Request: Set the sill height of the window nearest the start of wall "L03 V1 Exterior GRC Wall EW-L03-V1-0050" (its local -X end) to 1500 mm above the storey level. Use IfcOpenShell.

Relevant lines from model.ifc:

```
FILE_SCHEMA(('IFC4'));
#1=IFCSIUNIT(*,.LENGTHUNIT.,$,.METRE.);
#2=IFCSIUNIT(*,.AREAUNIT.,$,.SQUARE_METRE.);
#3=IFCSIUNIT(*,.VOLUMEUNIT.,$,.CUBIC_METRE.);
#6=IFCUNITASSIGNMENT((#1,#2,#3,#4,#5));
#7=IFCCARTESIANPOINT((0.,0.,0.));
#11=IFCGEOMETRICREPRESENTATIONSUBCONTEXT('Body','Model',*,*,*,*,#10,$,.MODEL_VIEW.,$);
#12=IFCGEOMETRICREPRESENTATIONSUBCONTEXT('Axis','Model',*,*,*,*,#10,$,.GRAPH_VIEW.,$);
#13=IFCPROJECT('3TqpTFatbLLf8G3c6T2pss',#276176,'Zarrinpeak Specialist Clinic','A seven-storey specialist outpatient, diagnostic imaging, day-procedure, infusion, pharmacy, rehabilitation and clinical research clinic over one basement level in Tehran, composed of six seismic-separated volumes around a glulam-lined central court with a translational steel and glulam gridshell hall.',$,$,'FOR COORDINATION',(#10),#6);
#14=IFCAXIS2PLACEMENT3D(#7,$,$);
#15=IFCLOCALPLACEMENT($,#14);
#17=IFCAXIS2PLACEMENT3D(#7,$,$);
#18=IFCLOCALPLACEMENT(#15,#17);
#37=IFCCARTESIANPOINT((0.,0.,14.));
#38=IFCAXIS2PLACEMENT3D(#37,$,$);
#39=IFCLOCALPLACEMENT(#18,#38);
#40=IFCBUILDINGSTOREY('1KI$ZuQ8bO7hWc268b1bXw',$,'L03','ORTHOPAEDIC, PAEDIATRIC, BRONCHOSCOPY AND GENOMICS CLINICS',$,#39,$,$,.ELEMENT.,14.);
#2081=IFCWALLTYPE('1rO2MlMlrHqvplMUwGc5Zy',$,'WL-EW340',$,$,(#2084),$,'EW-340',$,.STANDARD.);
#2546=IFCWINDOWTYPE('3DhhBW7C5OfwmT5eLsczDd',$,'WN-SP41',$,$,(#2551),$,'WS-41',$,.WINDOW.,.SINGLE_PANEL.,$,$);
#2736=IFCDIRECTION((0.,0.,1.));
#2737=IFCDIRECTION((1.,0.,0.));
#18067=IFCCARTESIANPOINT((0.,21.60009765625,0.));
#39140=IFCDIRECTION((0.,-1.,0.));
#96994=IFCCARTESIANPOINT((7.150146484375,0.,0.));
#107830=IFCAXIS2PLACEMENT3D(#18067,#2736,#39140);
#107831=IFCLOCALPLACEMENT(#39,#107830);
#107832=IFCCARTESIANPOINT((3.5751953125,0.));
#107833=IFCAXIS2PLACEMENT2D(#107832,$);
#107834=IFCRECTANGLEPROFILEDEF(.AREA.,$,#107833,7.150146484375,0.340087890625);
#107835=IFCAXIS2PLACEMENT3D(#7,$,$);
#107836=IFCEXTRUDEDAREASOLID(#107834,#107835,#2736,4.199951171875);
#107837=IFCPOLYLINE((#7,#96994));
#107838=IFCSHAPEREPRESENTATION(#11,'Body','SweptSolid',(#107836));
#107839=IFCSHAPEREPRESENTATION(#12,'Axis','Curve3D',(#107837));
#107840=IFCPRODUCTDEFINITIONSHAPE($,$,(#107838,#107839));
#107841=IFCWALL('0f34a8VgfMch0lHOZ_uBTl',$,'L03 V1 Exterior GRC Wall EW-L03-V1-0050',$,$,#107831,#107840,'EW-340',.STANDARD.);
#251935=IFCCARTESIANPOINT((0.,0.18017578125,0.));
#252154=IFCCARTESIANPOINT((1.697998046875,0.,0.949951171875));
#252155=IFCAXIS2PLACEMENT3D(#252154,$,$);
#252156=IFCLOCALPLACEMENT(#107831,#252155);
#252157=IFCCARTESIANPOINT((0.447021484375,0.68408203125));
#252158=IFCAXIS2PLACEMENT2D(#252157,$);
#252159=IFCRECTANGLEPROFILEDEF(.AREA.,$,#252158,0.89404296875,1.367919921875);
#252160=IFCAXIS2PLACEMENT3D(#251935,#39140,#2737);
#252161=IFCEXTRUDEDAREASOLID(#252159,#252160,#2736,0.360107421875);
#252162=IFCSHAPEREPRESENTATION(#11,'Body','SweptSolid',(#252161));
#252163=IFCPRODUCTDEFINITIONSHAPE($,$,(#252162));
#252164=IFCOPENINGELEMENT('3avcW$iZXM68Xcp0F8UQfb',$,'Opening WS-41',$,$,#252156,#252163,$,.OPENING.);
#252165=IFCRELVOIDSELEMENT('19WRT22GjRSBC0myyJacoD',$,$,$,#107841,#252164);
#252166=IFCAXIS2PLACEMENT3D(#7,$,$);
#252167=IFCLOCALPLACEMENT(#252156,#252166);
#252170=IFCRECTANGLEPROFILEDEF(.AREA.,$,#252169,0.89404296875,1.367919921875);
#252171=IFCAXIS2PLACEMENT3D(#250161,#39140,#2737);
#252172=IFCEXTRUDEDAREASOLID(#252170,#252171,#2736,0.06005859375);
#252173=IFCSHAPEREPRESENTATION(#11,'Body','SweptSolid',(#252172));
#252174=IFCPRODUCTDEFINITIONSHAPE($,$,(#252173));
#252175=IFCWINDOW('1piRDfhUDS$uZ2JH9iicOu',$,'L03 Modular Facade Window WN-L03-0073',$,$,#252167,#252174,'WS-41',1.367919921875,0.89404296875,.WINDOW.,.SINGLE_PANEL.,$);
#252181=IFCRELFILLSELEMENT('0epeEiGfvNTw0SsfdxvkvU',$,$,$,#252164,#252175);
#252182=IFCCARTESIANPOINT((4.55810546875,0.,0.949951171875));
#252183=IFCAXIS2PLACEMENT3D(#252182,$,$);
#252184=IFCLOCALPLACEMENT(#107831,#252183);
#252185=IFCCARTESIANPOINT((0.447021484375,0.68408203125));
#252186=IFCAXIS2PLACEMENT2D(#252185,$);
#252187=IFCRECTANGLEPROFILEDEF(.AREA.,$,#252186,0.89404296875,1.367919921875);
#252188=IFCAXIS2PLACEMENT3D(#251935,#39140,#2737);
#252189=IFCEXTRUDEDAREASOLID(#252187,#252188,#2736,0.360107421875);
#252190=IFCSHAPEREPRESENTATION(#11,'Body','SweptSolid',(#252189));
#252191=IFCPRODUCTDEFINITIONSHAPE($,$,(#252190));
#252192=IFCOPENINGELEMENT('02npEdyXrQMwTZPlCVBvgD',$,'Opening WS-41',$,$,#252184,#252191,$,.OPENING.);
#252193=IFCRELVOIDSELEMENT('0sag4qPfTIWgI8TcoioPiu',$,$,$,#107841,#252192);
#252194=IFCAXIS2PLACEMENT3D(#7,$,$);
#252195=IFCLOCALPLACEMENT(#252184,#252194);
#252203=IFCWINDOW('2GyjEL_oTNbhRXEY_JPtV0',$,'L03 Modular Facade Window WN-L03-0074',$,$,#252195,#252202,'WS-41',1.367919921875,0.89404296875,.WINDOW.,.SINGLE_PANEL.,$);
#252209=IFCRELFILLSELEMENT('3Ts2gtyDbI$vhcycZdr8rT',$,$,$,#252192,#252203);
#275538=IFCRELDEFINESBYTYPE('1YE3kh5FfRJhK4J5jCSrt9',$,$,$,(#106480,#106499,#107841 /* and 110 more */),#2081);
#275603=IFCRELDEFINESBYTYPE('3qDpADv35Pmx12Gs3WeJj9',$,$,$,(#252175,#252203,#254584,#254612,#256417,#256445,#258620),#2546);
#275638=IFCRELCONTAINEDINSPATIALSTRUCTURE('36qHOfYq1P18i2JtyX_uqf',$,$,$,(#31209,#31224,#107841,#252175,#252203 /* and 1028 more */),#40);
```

```python
import numpy as np
import ifcopenshell
import ifcopenshell.api.geometry
import ifcopenshell.geom
import ifcopenshell.util.element
import ifcopenshell.util.placement
import ifcopenshell.util.shape
import ifcopenshell.util.unit

model = ifcopenshell.open("model.ifc")
unit_scale = ifcopenshell.util.unit.calculate_unit_scale(model)

window = model.by_guid("1piRDfhUDS$uZ2JH9iicOu")
opening = window.FillsVoids[0].RelatingOpeningElement
storey = ifcopenshell.util.element.get_container(window, ifc_class="IfcBuildingStorey")
level = ifcopenshell.util.placement.get_local_placement(storey.ObjectPlacement)[2, 3]

# The opening's origin need not be at the sill, so measure its lowest point.
shape = ifcopenshell.geom.create_shape(ifcopenshell.geom.settings(), opening)
bottom = ifcopenshell.util.shape.get_shape_bottom_elevation(shape, shape.geometry) / unit_scale
dz = level + 1.5 / unit_scale - bottom

shift = np.array([0.0, 0.0, dz])
# The window is placed relative to its opening, so it follows when the opening moves.
matrix = ifcopenshell.util.placement.get_local_placement(opening.ObjectPlacement)
matrix[:3, 3] += shift
ifcopenshell.api.geometry.edit_object_placement(
    model, product=opening, matrix=matrix, is_si=False, should_transform_children=True
)

print(f"moved by {dz * unit_scale:+.3f} m")

model.write("model_v2.ifc")
```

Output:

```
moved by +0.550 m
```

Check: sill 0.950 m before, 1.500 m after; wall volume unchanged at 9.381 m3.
